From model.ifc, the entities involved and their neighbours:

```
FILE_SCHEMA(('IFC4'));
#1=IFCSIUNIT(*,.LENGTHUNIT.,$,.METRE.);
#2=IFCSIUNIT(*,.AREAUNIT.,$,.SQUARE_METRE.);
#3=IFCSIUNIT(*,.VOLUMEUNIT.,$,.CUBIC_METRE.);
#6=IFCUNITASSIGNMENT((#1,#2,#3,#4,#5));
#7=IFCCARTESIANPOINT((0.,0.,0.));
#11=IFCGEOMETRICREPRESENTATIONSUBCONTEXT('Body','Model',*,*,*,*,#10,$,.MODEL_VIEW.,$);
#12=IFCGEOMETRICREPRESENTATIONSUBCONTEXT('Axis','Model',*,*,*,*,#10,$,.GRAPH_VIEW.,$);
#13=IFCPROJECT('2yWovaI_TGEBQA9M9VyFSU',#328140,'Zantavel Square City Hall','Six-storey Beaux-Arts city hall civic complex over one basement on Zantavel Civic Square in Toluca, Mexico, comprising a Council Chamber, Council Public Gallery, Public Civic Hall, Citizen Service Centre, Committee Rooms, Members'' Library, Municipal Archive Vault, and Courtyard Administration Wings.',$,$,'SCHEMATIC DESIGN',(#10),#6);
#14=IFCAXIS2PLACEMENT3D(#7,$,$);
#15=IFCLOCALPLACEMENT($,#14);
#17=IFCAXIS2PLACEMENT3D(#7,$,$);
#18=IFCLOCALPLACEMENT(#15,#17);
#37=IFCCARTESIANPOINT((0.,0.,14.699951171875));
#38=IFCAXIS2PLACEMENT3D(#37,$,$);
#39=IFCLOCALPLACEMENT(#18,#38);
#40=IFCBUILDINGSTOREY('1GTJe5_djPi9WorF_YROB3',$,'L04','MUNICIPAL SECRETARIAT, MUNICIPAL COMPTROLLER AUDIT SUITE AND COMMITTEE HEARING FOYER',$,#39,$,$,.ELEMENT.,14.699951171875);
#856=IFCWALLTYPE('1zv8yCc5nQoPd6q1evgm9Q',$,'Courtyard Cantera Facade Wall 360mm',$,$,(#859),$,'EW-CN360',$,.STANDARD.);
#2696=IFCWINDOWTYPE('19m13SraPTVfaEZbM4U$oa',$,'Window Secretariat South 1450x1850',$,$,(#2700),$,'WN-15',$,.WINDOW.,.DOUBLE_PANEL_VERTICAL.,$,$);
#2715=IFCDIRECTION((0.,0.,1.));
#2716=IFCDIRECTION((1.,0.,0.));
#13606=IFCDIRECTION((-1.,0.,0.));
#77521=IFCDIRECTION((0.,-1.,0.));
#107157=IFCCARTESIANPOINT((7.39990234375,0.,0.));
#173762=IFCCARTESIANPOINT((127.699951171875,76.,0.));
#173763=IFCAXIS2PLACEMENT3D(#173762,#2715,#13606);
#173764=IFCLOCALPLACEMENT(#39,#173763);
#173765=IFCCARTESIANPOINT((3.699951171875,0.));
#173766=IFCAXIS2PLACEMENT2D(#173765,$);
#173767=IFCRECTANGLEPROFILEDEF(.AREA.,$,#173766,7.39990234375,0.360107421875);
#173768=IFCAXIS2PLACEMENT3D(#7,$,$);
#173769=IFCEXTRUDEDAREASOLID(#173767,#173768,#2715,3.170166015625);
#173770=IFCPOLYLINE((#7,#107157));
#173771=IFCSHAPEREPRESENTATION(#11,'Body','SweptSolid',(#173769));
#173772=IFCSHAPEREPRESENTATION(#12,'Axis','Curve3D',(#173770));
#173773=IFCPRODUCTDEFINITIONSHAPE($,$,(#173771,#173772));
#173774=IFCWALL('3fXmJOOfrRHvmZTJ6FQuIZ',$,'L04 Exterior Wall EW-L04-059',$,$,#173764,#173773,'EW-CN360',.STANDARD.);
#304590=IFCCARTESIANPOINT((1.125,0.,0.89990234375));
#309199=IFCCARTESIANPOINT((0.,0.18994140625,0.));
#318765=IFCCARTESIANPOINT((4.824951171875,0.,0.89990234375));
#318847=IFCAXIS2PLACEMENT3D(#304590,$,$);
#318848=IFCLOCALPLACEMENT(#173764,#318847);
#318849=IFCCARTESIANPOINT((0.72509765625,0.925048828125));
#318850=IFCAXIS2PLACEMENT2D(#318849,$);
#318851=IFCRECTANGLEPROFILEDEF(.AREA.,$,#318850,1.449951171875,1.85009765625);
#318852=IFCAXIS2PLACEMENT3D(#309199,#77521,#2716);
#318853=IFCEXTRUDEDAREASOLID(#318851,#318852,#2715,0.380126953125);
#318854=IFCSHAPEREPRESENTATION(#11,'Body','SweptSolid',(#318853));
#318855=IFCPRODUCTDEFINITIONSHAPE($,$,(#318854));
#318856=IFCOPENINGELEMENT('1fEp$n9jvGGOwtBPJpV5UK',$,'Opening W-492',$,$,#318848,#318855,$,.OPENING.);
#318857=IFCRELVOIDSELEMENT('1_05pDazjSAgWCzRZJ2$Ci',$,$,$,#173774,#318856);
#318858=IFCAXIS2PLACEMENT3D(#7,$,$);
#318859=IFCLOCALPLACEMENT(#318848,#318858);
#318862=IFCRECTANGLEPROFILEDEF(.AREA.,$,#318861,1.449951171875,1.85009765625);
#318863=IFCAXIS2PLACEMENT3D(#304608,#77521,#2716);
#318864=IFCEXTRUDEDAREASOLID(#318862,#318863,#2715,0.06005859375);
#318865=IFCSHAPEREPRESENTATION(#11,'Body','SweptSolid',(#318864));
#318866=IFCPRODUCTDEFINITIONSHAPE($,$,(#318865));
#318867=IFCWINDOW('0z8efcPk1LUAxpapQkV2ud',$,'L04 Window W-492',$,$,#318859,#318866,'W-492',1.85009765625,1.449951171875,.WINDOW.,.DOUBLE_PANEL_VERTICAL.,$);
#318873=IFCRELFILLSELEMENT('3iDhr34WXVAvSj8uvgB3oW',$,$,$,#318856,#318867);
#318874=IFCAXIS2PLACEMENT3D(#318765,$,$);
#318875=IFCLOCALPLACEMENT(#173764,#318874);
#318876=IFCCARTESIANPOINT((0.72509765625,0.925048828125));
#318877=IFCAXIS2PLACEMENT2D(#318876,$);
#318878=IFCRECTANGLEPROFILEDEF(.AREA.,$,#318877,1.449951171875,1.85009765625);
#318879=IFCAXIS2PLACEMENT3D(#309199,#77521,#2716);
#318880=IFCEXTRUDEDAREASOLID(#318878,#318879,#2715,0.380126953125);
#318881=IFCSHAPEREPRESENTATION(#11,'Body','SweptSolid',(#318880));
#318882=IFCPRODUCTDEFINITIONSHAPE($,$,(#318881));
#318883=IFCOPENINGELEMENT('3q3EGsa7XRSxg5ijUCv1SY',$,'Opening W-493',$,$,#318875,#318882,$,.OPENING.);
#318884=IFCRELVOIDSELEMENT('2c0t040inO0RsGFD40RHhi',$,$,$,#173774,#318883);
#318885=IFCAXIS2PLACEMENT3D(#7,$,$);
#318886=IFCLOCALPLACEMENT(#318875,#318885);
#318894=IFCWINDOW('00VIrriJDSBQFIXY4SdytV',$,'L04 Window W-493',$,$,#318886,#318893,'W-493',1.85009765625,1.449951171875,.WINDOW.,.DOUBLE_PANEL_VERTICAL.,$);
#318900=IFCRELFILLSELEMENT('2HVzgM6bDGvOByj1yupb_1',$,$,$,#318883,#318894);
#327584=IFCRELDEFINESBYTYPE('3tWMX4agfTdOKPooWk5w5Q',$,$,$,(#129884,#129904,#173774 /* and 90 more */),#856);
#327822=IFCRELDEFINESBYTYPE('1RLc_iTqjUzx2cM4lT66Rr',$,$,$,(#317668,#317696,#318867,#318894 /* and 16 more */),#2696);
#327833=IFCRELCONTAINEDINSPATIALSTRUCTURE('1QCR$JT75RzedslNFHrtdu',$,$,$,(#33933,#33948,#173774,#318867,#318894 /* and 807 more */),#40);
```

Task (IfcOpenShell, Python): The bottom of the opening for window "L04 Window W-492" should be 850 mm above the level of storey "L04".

```python
import numpy as np
import ifcopenshell
import ifcopenshell.api.geometry
import ifcopenshell.geom
import ifcopenshell.util.element
import ifcopenshell.util.placement
import ifcopenshell.util.shape
import ifcopenshell.util.unit

model = ifcopenshell.open("model.ifc")
unit_scale = ifcopenshell.util.unit.calculate_unit_scale(model)

window = model.by_guid("0z8efcPk1LUAxpapQkV2ud")
opening = window.FillsVoids[0].RelatingOpeningElement
storey = ifcopenshell.util.element.get_container(window, ifc_class="IfcBuildingStorey")
level = ifcopenshell.util.placement.get_local_placement(storey.ObjectPlacement)[2, 3]

# The opening's origin need not be at the sill, so measure its lowest point.
shape = ifcopenshell.geom.create_shape(ifcopenshell.geom.settings(), opening)
bottom = ifcopenshell.util.shape.get_shape_bottom_elevation(shape, shape.geometry) / unit_scale
dz = level + 0.85 / unit_scale - bottom

shift = np.array([0.0, 0.0, dz])
# The window is placed relative to its opening, so it follows when the opening moves.
matrix = ifcopenshell.util.placement.get_local_placement(opening.ObjectPlacement)
matrix[:3, 3] += shift
ifcopenshell.api.geometry.edit_object_placement(
    model, product=opening, matrix=matrix, is_si=False, should_transform_children=True
)

print(f"moved by {dz * unit_scale:+.3f} m")

model.write("model_rev.ifc")
```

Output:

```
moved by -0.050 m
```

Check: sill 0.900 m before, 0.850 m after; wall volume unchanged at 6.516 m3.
